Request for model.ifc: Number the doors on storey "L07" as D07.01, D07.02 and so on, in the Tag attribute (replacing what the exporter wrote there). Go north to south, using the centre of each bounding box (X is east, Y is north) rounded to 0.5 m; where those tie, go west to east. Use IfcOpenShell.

First a look at what the model holds.

```python
import ifcopenshell
import ifcopenshell.util.element
import ifcopenshell.util.placement

model = ifcopenshell.open("model.ifc")
print(model.schema)
storey = next(s for s in model.by_type("IfcBuildingStorey") if s.Name == "L07")
doors = [e for e in ifcopenshell.util.element.get_decomposition(storey) if e.is_a("IfcDoor")]
for e in sorted(doors, key=lambda e: e.id()):
    origin = ifcopenshell.util.placement.get_local_placement(e.ObjectPlacement)[:3, 3]
    print(e.id(), e.Tag, e.Name, origin.round(2) + 0.0, sep=" | ")
```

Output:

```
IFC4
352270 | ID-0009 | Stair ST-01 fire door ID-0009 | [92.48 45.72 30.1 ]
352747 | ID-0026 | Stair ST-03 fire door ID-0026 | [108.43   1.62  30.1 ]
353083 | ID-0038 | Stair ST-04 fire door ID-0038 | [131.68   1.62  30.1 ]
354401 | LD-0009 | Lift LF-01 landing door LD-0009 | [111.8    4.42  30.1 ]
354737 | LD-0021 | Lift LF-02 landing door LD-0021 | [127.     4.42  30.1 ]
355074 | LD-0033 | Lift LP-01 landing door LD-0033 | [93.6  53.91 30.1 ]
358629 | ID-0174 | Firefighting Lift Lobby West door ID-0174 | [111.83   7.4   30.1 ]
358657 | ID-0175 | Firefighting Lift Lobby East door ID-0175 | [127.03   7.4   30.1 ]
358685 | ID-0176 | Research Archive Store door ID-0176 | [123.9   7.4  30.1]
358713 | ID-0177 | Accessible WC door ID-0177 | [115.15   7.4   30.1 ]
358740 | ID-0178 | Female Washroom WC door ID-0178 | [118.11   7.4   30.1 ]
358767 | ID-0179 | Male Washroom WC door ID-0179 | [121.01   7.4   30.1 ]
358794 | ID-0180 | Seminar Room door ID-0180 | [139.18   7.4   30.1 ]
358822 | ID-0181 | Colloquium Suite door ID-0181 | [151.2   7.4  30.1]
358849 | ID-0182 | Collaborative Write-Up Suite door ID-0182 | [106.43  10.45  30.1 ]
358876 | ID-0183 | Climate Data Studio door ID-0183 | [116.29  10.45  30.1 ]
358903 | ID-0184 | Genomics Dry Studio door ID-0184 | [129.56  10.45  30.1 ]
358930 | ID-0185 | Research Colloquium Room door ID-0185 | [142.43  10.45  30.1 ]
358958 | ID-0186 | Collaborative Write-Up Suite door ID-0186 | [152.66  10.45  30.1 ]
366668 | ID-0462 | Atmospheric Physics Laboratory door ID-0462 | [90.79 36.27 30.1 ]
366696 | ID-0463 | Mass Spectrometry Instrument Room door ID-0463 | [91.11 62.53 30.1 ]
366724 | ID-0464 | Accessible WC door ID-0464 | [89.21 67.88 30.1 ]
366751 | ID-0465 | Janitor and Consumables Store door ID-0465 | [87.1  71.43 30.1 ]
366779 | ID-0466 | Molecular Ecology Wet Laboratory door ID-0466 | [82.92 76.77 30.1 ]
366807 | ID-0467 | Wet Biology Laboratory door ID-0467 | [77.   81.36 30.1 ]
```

```python
import ifcopenshell
import ifcopenshell.geom
import ifcopenshell.util.element
import ifcopenshell.util.shape

model = ifcopenshell.open("model.ifc")
settings = ifcopenshell.geom.settings()
settings.set("use-world-coords", True)


def centre(element):
    shape = ifcopenshell.geom.create_shape(settings, element)
    return ifcopenshell.util.shape.get_bbox_centroid(shape.geometry)


storey = next(s for s in model.by_type("IfcBuildingStorey") if s.Name == "L07")
doors = [e for e in ifcopenshell.util.element.get_decomposition(storey) if e.is_a("IfcDoor")]

# Insertion points can sit at a corner or the storey origin, so sort by the geometry (in metres).
centres = {e: centre(e) for e in doors}
doors.sort(key=lambda e: (-round(centres[e][1] / 0.5), centres[e][0]))

for i, e in enumerate(doors, start=1):
    number = f"D07.{i:02d}"
    e.Tag = number
    print(e.id(), number)

model.write("model-out.ifc")
```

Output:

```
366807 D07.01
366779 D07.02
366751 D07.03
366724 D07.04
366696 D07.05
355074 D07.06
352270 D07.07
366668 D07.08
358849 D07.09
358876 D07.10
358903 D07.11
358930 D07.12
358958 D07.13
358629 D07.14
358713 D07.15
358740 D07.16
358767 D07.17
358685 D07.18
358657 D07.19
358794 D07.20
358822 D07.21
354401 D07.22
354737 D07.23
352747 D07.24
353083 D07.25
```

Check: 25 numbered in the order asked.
